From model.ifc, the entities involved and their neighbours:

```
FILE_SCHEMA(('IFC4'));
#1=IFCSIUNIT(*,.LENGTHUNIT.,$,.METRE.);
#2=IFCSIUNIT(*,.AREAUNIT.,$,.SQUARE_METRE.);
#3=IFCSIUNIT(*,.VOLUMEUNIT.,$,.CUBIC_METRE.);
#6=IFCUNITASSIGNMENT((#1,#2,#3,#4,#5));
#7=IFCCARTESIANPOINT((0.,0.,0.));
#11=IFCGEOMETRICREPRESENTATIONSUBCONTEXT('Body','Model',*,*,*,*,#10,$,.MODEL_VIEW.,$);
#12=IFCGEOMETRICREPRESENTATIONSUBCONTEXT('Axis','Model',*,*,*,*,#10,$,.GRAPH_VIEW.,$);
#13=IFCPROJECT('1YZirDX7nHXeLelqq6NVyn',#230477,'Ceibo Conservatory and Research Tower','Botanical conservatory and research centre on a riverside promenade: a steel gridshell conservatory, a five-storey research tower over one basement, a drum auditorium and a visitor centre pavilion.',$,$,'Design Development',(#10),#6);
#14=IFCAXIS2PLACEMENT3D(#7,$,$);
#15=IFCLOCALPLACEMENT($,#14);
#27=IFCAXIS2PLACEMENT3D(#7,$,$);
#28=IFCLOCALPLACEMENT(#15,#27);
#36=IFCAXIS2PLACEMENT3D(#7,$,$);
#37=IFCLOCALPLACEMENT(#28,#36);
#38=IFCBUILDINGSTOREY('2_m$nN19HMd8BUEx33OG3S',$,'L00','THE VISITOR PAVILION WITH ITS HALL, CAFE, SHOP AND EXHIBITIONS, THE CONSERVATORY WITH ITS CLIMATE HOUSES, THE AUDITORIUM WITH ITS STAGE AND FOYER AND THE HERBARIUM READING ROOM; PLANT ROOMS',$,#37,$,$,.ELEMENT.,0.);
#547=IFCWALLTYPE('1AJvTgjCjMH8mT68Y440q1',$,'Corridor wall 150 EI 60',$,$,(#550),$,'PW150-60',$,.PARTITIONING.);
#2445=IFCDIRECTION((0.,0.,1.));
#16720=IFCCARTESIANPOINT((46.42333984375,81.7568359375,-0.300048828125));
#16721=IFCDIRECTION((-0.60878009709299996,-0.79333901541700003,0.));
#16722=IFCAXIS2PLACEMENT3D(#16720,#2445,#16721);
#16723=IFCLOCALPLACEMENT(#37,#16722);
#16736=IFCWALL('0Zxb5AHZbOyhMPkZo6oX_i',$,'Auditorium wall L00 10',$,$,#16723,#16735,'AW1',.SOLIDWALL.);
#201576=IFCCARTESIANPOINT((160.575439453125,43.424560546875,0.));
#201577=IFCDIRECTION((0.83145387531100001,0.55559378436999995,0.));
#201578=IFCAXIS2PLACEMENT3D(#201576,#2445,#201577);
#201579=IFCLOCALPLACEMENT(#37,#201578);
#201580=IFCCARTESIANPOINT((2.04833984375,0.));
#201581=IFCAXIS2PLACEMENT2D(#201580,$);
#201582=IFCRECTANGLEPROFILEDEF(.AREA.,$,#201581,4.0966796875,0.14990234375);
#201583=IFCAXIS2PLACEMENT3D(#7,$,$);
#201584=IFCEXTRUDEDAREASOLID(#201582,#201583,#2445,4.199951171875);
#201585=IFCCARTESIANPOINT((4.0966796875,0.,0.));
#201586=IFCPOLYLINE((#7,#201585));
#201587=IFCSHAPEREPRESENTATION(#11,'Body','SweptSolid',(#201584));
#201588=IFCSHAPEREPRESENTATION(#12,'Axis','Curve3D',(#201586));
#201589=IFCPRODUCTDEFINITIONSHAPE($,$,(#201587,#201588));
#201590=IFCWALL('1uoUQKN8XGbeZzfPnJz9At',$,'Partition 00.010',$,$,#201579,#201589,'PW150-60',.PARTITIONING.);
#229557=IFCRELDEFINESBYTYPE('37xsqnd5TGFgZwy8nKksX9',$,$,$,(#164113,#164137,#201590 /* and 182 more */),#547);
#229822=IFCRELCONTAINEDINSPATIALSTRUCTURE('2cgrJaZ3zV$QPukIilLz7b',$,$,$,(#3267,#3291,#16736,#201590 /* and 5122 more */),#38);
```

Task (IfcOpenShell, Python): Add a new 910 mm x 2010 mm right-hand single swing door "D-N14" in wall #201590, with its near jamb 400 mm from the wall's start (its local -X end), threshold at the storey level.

```python
import numpy as np
import ifcopenshell
import ifcopenshell.api.feature
import ifcopenshell.api.geometry
import ifcopenshell.api.root
import ifcopenshell.api.spatial
import ifcopenshell.geom
import ifcopenshell.util.element
import ifcopenshell.util.placement
import ifcopenshell.util.representation
import ifcopenshell.util.shape
import ifcopenshell.util.unit

model = ifcopenshell.open("model.ifc")
unit_scale = ifcopenshell.util.unit.calculate_unit_scale(model)
settings = ifcopenshell.geom.settings()


def volume(element):
    """Net volume in cubic metres, openings subtracted."""
    shape = ifcopenshell.geom.create_shape(settings, element)
    return ifcopenshell.util.shape.get_volume(shape.geometry)


wall = model.by_guid("1uoUQKN8XGbeZzfPnJz9At")
storey = ifcopenshell.util.element.get_container(wall, ifc_class="IfcBuildingStorey")
context = ifcopenshell.util.representation.get_context(model, "Model", "Body", "MODEL_VIEW")
before = volume(wall)

width, height, from_end, sill = 0.91, 2.01, 0.4, 0.0  # metres

# The wall runs along its own X axis, and the end named is its -X end.
wall_shape = ifcopenshell.geom.create_shape(settings, wall)
x, y, z = ifcopenshell.util.shape.get_vertices(wall_shape.geometry).T
start = x.min() + from_end
face, thickness = float(y.min()), float(y.max() - y.min())
wall_matrix = ifcopenshell.util.placement.get_local_placement(wall.ObjectPlacement)
level = ifcopenshell.util.placement.get_local_placement(storey.ObjectPlacement)[2, 3]


def in_wall(x, y):
    """Placement at x, y metres in the wall's axes, at sill height."""
    matrix = wall_matrix.copy()
    matrix[:, 3] = wall_matrix @ np.array([x / unit_scale, y / unit_scale, 0.0, 1.0])
    matrix[2, 3] = level + sill / unit_scale
    return matrix


# Opening: a box that overshoots both wall faces by 50 mm.
opening = ifcopenshell.api.root.create_entity(model, ifc_class="IfcOpeningElement", predefined_type="OPENING")
box = ifcopenshell.api.geometry.add_wall_representation(
    model, context=context, length=width, height=height, thickness=thickness + 0.1
)
ifcopenshell.api.geometry.assign_representation(model, product=opening, representation=box)
ifcopenshell.api.geometry.edit_object_placement(model, product=opening, matrix=in_wall(start, face - 0.05), is_si=False)
ifcopenshell.api.feature.add_feature(model, feature=opening, element=wall)

door = ifcopenshell.api.root.create_entity(model, ifc_class="IfcDoor", name="D-N14", predefined_type="DOOR")
door.OverallWidth, door.OverallHeight = width / unit_scale, height / unit_scale
door.OperationType = "SINGLE_SWING_RIGHT"
body = ifcopenshell.api.geometry.add_door_representation(
    model,
    context=context,
    overall_width=door.OverallWidth,
    overall_height=door.OverallHeight,
    operation_type="SINGLE_SWING_RIGHT",
    lining_properties={"LiningDepth": thickness / unit_scale, "ThresholdDepth": thickness / unit_scale},
)
ifcopenshell.api.geometry.assign_representation(model, product=door, representation=body)
ifcopenshell.api.spatial.assign_container(model, products=[door], relating_structure=storey)
ifcopenshell.api.feature.add_filling(model, opening=opening, element=door)

# The lining spans the wall, so the door starts at the wall face.
ifcopenshell.api.geometry.edit_object_placement(model, product=door, matrix=in_wall(start, face), is_si=False)

after = volume(wall)

print(f"wall volume {before:.3f} -> {after:.3f} m3")

model.write("model-out.ifc")
```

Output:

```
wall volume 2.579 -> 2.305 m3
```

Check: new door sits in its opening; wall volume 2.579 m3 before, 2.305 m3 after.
